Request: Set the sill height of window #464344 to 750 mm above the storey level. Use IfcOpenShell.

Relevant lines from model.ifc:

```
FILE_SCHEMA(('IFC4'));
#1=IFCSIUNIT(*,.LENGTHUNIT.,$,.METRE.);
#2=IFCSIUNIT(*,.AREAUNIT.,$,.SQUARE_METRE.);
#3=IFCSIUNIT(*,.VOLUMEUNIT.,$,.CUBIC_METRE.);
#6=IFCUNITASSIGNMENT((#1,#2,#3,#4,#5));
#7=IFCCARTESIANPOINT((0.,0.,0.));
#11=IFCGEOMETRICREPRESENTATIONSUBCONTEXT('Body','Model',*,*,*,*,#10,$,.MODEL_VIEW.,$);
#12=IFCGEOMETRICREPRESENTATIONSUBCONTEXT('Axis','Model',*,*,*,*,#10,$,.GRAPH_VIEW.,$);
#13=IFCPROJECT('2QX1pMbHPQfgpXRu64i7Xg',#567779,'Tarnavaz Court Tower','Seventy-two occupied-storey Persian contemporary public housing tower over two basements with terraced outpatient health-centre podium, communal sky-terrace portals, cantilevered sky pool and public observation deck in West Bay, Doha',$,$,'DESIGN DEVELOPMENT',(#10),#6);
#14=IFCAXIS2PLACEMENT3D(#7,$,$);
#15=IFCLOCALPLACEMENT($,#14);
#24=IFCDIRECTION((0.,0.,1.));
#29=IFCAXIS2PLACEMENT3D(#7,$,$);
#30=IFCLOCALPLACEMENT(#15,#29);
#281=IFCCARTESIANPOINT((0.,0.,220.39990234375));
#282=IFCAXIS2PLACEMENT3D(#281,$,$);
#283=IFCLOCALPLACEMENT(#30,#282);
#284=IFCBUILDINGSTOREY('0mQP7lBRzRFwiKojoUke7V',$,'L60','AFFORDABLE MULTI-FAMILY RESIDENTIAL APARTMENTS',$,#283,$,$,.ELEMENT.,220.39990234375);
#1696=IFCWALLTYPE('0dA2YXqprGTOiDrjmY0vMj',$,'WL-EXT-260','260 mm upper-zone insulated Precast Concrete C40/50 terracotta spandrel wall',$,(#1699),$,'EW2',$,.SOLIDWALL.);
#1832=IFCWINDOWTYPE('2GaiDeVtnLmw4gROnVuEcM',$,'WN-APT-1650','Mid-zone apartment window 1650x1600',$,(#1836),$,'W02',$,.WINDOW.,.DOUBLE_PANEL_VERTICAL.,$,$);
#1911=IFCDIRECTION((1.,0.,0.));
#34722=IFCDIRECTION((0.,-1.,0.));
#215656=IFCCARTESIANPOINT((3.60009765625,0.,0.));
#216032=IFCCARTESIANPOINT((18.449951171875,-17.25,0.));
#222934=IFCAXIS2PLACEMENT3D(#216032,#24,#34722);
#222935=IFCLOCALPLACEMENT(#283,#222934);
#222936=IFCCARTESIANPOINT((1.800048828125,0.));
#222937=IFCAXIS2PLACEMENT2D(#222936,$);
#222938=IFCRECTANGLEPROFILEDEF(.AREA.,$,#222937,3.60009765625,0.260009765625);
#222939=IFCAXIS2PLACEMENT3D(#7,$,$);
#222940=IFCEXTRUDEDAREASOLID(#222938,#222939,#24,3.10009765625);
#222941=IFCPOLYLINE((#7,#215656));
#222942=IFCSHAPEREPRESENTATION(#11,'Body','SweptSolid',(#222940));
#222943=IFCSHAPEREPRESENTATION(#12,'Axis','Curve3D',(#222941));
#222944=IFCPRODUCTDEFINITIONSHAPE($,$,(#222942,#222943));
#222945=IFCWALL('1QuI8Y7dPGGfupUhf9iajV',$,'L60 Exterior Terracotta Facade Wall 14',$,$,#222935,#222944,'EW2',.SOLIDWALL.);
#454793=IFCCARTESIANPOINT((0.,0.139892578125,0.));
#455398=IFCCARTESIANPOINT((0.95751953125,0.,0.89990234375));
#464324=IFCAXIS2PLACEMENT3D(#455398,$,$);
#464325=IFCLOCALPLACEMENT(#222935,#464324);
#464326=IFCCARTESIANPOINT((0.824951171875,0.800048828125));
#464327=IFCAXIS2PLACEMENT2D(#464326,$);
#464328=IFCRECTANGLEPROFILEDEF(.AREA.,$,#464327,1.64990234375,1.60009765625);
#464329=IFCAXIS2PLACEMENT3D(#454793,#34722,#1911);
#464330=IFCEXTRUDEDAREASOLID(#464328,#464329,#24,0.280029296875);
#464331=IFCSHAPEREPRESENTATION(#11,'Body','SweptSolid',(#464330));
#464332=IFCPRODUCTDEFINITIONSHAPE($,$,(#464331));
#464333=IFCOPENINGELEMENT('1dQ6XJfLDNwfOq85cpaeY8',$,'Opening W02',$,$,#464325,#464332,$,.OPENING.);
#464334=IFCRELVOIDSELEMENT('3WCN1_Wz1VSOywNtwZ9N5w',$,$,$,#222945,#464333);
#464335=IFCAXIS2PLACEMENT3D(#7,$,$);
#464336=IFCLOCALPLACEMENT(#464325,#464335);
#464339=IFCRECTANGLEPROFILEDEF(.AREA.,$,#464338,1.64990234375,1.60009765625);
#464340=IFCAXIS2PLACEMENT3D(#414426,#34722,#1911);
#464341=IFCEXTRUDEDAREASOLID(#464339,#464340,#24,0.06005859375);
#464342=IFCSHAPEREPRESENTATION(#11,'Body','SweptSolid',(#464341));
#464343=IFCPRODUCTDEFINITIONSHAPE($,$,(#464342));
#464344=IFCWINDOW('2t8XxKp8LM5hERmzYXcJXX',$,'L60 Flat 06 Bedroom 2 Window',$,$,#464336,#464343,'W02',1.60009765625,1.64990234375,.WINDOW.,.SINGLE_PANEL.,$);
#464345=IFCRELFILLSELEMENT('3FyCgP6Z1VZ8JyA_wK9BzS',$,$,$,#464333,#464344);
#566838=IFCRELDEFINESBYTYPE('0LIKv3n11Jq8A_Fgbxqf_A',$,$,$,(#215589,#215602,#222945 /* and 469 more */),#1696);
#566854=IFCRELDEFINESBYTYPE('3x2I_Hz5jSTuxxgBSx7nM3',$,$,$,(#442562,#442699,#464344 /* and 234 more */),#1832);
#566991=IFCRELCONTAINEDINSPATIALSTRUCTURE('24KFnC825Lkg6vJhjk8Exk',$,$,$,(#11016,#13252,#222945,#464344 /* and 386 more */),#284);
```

```python
import numpy as np
import ifcopenshell
import ifcopenshell.api.geometry
import ifcopenshell.geom
import ifcopenshell.util.element
import ifcopenshell.util.placement
import ifcopenshell.util.shape
import ifcopenshell.util.unit

model = ifcopenshell.open("model.ifc")
unit_scale = ifcopenshell.util.unit.calculate_unit_scale(model)

window = model.by_guid("2t8XxKp8LM5hERmzYXcJXX")
opening = window.FillsVoids[0].RelatingOpeningElement
storey = ifcopenshell.util.element.get_container(window, ifc_class="IfcBuildingStorey")
level = ifcopenshell.util.placement.get_local_placement(storey.ObjectPlacement)[2, 3]

# The opening's origin need not be at the sill, so measure its lowest point.
shape = ifcopenshell.geom.create_shape(ifcopenshell.geom.settings(), opening)
bottom = ifcopenshell.util.shape.get_shape_bottom_elevation(shape, shape.geometry) / unit_scale
dz = level + 0.75 / unit_scale - bottom

shift = np.array([0.0, 0.0, dz])
# The window is placed relative to its opening, so it follows when the opening moves.
matrix = ifcopenshell.util.placement.get_local_placement(opening.ObjectPlacement)
matrix[:3, 3] += shift
ifcopenshell.api.geometry.edit_object_placement(
    model, product=opening, matrix=matrix, is_si=False, should_transform_children=True
)

print(f"moved by {dz * unit_scale:+.3f} m")

model.write("model_rev.ifc")
```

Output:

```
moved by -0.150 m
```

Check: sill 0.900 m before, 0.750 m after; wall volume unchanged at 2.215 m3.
